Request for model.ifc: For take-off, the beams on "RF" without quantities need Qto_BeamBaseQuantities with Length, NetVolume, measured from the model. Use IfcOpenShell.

First a look at what the model holds.

```python
import ifcopenshell
import ifcopenshell.util.element
import ifcopenshell.util.unit

model = ifcopenshell.open("model.ifc")
print(model.schema)
for unit_type in ("LENGTHUNIT", "AREAUNIT", "VOLUMEUNIT"):
    print(unit_type, ifcopenshell.util.unit.calculate_unit_scale(model, unit_type))
storey = next(s for s in model.by_type("IfcBuildingStorey") if s.Name == "RF")
beams = [e for e in ifcopenshell.util.element.get_decomposition(storey) if e.is_a("IfcBeam")]
for e in sorted(beams, key=lambda e: e.id()):
    print(e.id(), e.is_a(), e.Name, list(ifcopenshell.util.element.get_psets(e, qtos_only=True)), sep=" | ")
```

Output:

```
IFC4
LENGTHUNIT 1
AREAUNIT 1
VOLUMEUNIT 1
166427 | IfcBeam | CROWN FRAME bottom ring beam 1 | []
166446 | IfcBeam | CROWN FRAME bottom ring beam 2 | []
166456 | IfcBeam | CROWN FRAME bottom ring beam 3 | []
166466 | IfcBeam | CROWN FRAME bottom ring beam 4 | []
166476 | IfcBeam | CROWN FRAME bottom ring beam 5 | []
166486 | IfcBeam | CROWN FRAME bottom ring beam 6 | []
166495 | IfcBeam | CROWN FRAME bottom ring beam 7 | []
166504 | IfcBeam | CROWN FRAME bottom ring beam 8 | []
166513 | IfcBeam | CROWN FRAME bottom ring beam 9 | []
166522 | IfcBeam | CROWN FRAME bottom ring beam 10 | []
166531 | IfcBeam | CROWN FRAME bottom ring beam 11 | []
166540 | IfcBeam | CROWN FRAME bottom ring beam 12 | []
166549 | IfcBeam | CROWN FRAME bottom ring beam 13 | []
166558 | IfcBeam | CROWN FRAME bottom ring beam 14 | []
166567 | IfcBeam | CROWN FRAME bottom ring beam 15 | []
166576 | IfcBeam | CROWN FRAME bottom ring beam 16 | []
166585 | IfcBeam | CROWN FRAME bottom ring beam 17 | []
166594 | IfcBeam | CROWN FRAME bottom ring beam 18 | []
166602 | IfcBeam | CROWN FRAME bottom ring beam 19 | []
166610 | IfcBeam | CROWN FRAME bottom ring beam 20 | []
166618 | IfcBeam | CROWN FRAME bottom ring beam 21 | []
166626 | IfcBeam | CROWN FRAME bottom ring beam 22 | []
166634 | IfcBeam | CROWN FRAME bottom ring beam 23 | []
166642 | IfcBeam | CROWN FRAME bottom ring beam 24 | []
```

```python
import ifcopenshell
import ifcopenshell.api.pset
import ifcopenshell.geom
import ifcopenshell.util.element
import ifcopenshell.util.shape
import ifcopenshell.util.unit

model = ifcopenshell.open("model.ifc")
unit_scale = ifcopenshell.util.unit.calculate_unit_scale(model)
volume_scale = ifcopenshell.util.unit.calculate_unit_scale(model, "VOLUMEUNIT")
settings = ifcopenshell.geom.settings()

storey = next(s for s in model.by_type("IfcBuildingStorey") if s.Name == "RF")
beams = [e for e in ifcopenshell.util.element.get_decomposition(storey) if e.is_a("IfcBeam")]

for e in sorted(beams, key=lambda e: e.id()):
    if ifcopenshell.util.element.get_psets(e, qtos_only=True, should_inherit=False):
        continue
    # Geometry comes back in metres, in the element's own axes.
    shape = ifcopenshell.geom.create_shape(settings, e)
    values = {
        "Length": ifcopenshell.util.shape.get_max_xyz(shape.geometry) / unit_scale,
        "NetVolume": ifcopenshell.util.shape.get_volume(shape.geometry) / volume_scale,
    }
    qto = ifcopenshell.api.pset.add_qto(model, product=e, name="Qto_BeamBaseQuantities")
    ifcopenshell.api.pset.edit_qto(model, qto=qto, properties=values)
    print(e.id(), {k: round(v, 3) for k, v in values.items()})

model.write("model_rev.ifc")
```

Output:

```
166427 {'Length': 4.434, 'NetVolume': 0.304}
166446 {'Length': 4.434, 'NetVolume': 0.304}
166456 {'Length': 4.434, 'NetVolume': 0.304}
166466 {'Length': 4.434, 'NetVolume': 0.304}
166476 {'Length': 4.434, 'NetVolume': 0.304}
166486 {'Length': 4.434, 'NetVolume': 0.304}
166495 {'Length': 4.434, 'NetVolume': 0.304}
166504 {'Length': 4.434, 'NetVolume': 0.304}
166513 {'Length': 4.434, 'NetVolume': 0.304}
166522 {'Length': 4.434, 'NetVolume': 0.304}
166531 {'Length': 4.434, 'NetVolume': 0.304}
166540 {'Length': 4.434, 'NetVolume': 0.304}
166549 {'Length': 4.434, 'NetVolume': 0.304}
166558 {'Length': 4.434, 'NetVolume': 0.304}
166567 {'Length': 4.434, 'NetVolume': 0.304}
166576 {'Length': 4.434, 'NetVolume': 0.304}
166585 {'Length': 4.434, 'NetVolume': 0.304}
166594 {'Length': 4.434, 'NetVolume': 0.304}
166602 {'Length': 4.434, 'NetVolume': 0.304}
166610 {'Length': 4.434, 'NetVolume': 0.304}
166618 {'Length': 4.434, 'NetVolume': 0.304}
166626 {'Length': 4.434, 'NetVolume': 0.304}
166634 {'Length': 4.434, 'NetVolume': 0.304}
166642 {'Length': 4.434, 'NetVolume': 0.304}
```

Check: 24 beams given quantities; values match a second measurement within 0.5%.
